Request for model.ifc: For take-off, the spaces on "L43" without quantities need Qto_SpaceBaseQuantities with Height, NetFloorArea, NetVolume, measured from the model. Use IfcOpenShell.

First a look at what the model holds.

```python
import ifcopenshell
import ifcopenshell.util.element
import ifcopenshell.util.unit

model = ifcopenshell.open("model.ifc")
print(model.schema)
for unit_type in ("LENGTHUNIT", "AREAUNIT", "VOLUMEUNIT"):
    print(unit_type, ifcopenshell.util.unit.calculate_unit_scale(model, unit_type))
storey = next(s for s in model.by_type("IfcBuildingStorey") if s.Name == "L43")
spaces = [e for e in ifcopenshell.util.element.get_decomposition(storey) if e.is_a("IfcSpace")]
for e in sorted(spaces, key=lambda e: e.id()):
    print(e.id(), e.is_a(), e.Name, list(ifcopenshell.util.element.get_psets(e, qtos_only=True)), sep=" | ")
```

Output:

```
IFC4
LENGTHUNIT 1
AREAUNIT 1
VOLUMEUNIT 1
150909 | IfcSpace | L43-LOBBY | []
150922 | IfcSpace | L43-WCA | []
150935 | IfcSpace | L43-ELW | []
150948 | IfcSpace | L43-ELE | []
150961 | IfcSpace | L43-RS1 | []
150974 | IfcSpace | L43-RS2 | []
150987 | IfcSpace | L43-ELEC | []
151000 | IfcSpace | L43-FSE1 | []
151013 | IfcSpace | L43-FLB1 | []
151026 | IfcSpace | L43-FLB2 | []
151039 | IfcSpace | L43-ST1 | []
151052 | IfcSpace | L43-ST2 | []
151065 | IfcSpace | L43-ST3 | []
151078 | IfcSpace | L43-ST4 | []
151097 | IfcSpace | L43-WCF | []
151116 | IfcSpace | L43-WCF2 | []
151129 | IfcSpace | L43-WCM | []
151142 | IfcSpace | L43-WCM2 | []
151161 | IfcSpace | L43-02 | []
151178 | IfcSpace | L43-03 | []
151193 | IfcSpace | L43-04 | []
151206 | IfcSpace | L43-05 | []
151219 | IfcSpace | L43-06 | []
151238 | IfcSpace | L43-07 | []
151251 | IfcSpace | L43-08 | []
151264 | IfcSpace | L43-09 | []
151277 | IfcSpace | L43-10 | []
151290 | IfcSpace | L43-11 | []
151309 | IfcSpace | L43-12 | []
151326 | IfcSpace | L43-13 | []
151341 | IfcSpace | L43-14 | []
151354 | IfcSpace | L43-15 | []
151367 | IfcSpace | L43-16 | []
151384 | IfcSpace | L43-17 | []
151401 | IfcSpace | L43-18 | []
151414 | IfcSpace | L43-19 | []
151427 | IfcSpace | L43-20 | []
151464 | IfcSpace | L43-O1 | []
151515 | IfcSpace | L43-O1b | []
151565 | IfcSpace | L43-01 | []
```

```python
import ifcopenshell
import ifcopenshell.api.pset
import ifcopenshell.geom
import ifcopenshell.util.element
import ifcopenshell.util.shape
import ifcopenshell.util.unit

model = ifcopenshell.open("model.ifc")
unit_scale = ifcopenshell.util.unit.calculate_unit_scale(model)
area_scale = ifcopenshell.util.unit.calculate_unit_scale(model, "AREAUNIT")
volume_scale = ifcopenshell.util.unit.calculate_unit_scale(model, "VOLUMEUNIT")
settings = ifcopenshell.geom.settings()

storey = next(s for s in model.by_type("IfcBuildingStorey") if s.Name == "L43")
spaces = [e for e in ifcopenshell.util.element.get_decomposition(storey) if e.is_a("IfcSpace")]

for e in sorted(spaces, key=lambda e: e.id()):
    if ifcopenshell.util.element.get_psets(e, qtos_only=True, should_inherit=False):
        continue
    # Geometry comes back in metres, in the element's own axes.
    shape = ifcopenshell.geom.create_shape(settings, e)
    values = {
        "Height": ifcopenshell.util.shape.get_z(shape.geometry) / unit_scale,
        "NetFloorArea": ifcopenshell.util.shape.get_footprint_area(shape.geometry) / area_scale,
        "NetVolume": ifcopenshell.util.shape.get_volume(shape.geometry) / volume_scale,
    }
    qto = ifcopenshell.api.pset.add_qto(model, product=e, name="Qto_SpaceBaseQuantities")
    ifcopenshell.api.pset.edit_qto(model, qto=qto, properties=values)
    print(e.id(), {k: round(v, 3) for k, v in values.items()})

model.write("model_updated.ifc")
```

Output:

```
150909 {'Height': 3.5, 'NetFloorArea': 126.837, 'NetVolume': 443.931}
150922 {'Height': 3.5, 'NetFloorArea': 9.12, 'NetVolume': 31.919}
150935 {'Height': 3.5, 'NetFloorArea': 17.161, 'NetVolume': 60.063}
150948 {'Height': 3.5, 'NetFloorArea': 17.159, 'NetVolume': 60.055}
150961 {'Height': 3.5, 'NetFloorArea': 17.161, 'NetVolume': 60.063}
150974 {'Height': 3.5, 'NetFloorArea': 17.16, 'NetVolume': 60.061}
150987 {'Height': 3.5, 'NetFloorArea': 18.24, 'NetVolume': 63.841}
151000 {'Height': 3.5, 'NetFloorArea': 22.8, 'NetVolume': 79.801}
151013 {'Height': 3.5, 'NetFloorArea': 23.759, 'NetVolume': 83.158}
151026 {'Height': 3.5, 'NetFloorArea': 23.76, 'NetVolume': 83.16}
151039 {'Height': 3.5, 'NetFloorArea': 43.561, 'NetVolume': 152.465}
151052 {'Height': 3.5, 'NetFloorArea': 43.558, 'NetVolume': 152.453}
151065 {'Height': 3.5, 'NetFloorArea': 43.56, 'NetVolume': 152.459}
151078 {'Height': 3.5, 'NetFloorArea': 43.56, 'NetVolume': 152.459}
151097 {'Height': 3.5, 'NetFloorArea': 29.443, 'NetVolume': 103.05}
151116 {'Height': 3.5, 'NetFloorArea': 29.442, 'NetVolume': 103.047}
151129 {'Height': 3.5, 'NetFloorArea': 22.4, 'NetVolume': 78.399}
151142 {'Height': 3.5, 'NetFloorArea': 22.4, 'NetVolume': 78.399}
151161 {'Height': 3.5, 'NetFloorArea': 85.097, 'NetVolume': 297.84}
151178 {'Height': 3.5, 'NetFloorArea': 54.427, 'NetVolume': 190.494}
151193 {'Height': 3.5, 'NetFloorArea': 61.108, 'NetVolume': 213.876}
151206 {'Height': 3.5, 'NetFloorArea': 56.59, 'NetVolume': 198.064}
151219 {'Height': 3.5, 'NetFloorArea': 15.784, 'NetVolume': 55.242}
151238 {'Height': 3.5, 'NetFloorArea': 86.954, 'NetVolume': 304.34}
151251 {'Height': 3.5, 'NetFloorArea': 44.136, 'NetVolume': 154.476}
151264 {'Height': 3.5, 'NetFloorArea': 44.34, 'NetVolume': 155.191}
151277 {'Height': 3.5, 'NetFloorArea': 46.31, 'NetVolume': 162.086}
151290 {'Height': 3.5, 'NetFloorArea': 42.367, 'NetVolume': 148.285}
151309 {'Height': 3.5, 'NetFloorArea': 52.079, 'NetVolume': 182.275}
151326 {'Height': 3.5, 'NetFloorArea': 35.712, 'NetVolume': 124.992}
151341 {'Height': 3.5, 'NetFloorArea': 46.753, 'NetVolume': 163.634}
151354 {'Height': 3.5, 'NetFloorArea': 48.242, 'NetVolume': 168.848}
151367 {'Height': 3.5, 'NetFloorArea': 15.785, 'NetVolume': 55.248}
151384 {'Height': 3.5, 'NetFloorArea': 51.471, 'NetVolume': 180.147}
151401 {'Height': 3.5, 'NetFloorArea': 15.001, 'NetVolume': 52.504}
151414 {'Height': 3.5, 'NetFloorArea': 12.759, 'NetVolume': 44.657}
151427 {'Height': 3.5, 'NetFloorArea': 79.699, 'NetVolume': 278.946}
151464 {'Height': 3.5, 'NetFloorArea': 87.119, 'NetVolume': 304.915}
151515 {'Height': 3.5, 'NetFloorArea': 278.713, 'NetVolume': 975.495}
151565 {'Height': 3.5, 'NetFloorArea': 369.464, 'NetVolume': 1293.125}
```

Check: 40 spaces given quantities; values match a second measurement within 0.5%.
